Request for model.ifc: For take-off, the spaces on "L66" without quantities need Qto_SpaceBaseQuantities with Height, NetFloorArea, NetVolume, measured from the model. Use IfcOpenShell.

First a look at what the model holds.

```python
import ifcopenshell
import ifcopenshell.util.element
import ifcopenshell.util.unit

model = ifcopenshell.open("model.ifc")
print(model.schema)
for unit_type in ("LENGTHUNIT", "AREAUNIT", "VOLUMEUNIT"):
    print(unit_type, ifcopenshell.util.unit.calculate_unit_scale(model, unit_type))
storey = next(s for s in model.by_type("IfcBuildingStorey") if s.Name == "L66")
spaces = [e for e in ifcopenshell.util.element.get_decomposition(storey) if e.is_a("IfcSpace")]
for e in sorted(spaces, key=lambda e: e.id()):
    print(e.id(), e.is_a(), e.Name, list(ifcopenshell.util.element.get_psets(e, qtos_only=True)), sep=" | ")
```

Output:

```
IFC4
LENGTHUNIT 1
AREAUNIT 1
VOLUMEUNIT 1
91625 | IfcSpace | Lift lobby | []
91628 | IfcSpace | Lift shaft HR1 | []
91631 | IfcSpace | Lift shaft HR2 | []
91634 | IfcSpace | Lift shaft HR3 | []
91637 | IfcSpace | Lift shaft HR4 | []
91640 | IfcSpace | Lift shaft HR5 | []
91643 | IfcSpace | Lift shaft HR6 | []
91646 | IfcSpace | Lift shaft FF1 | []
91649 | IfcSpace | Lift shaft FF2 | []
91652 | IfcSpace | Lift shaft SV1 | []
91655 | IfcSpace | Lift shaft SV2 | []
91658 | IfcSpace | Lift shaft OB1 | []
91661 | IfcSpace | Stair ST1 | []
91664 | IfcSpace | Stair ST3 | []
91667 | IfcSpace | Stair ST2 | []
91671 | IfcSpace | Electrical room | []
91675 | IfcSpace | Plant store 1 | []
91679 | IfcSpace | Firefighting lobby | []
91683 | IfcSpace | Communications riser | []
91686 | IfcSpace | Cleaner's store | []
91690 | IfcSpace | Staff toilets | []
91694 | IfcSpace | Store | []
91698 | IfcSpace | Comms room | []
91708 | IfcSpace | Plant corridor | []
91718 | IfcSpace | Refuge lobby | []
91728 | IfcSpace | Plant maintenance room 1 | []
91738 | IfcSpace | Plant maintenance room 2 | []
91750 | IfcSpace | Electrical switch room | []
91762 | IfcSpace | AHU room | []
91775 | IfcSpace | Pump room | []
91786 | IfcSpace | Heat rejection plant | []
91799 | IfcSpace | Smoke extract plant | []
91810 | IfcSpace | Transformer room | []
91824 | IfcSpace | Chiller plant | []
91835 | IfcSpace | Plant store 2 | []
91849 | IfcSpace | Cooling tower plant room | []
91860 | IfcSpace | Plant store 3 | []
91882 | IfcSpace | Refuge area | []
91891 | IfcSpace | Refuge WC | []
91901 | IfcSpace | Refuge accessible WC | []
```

```python
import ifcopenshell
import ifcopenshell.api.pset
import ifcopenshell.geom
import ifcopenshell.util.element
import ifcopenshell.util.shape
import ifcopenshell.util.unit

model = ifcopenshell.open("model.ifc")
unit_scale = ifcopenshell.util.unit.calculate_unit_scale(model)
area_scale = ifcopenshell.util.unit.calculate_unit_scale(model, "AREAUNIT")
volume_scale = ifcopenshell.util.unit.calculate_unit_scale(model, "VOLUMEUNIT")
settings = ifcopenshell.geom.settings()

storey = next(s for s in model.by_type("IfcBuildingStorey") if s.Name == "L66")
spaces = [e for e in ifcopenshell.util.element.get_decomposition(storey) if e.is_a("IfcSpace")]

for e in sorted(spaces, key=lambda e: e.id()):
    if ifcopenshell.util.element.get_psets(e, qtos_only=True, should_inherit=False):
        continue
    # Geometry comes back in metres, in the element's own axes.
    shape = ifcopenshell.geom.create_shape(settings, e)
    values = {
        "Height": ifcopenshell.util.shape.get_z(shape.geometry) / unit_scale,
        "NetFloorArea": ifcopenshell.util.shape.get_footprint_area(shape.geometry) / area_scale,
        "NetVolume": ifcopenshell.util.shape.get_volume(shape.geometry) / volume_scale,
    }
    qto = ifcopenshell.api.pset.add_qto(model, product=e, name="Qto_SpaceBaseQuantities")
    ifcopenshell.api.pset.edit_qto(model, qto=qto, properties=values)
    print(e.id(), {k: round(v, 3) for k, v in values.items()})

model.write("model_updated.ifc")
```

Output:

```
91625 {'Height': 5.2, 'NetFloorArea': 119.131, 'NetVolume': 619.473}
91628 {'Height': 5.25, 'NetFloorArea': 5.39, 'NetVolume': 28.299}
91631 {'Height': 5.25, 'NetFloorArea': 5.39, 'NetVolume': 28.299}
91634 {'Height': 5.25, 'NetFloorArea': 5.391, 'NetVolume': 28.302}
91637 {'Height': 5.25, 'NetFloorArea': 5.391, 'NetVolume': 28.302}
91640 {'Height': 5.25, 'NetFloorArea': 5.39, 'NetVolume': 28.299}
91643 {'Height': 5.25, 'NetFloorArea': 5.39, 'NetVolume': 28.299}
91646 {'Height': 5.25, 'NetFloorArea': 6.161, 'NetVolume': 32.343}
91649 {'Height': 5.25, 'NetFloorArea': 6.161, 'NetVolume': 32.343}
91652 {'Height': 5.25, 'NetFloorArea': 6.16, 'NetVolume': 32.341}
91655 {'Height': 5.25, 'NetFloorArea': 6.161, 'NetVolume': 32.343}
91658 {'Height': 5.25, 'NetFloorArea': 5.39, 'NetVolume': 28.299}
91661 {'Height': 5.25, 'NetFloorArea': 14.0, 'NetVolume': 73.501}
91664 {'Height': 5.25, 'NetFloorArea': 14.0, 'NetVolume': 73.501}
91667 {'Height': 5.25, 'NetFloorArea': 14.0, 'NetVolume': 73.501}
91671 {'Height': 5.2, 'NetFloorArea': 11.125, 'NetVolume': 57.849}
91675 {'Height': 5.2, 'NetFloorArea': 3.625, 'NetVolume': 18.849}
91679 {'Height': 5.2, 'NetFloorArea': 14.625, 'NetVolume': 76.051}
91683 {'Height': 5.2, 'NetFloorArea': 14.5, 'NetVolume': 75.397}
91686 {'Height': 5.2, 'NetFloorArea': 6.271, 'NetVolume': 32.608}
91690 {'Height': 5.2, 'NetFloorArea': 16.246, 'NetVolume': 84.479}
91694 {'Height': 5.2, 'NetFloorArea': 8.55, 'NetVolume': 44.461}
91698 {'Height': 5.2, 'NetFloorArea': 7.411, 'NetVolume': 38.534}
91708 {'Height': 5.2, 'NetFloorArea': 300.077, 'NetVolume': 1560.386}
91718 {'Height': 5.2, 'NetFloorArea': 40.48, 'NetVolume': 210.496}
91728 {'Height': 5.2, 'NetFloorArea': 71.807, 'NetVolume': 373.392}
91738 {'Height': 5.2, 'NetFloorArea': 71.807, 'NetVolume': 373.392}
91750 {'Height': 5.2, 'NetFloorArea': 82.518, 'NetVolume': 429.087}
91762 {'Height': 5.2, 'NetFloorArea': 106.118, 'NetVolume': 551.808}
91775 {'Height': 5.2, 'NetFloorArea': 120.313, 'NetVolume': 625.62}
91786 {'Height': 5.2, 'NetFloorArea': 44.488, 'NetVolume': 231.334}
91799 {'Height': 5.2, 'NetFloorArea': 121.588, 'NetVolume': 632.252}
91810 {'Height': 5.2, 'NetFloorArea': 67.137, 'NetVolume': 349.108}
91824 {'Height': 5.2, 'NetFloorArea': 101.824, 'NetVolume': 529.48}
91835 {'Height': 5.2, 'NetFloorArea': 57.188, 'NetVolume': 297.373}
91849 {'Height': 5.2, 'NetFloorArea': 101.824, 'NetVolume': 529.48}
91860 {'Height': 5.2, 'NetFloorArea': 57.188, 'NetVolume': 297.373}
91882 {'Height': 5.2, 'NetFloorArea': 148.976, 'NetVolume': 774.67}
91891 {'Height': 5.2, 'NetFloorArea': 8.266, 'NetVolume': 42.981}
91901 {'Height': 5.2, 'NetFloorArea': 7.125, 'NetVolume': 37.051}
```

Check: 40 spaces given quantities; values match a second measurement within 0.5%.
